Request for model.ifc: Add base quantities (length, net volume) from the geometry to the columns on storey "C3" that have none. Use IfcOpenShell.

First a look at what the model holds.

```python
import ifcopenshell
import ifcopenshell.util.element
import ifcopenshell.util.unit

model = ifcopenshell.open("model.ifc")
print(model.schema)
for unit_type in ("LENGTHUNIT", "AREAUNIT", "VOLUMEUNIT"):
    print(unit_type, ifcopenshell.util.unit.calculate_unit_scale(model, unit_type))
storey = next(s for s in model.by_type("IfcBuildingStorey") if s.Name == "C3")
columns = [e for e in ifcopenshell.util.element.get_decomposition(storey) if e.is_a("IfcColumn")]
for e in sorted(columns, key=lambda e: e.id()):
    print(e.id(), e.is_a(), e.Name, list(ifcopenshell.util.element.get_psets(e, qtos_only=True)), sep=" | ")
```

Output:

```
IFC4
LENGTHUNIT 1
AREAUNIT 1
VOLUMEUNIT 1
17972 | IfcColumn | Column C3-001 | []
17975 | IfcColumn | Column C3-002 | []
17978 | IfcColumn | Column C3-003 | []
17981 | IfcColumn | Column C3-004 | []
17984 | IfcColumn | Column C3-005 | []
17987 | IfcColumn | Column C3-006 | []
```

```python
import ifcopenshell
import ifcopenshell.api.pset
import ifcopenshell.geom
import ifcopenshell.util.element
import ifcopenshell.util.shape
import ifcopenshell.util.unit

model = ifcopenshell.open("model.ifc")
unit_scale = ifcopenshell.util.unit.calculate_unit_scale(model)
volume_scale = ifcopenshell.util.unit.calculate_unit_scale(model, "VOLUMEUNIT")
settings = ifcopenshell.geom.settings()

storey = next(s for s in model.by_type("IfcBuildingStorey") if s.Name == "C3")
columns = [e for e in ifcopenshell.util.element.get_decomposition(storey) if e.is_a("IfcColumn")]

for e in sorted(columns, key=lambda e: e.id()):
    if ifcopenshell.util.element.get_psets(e, qtos_only=True, should_inherit=False):
        continue
    # Geometry comes back in metres, in the element's own axes.
    shape = ifcopenshell.geom.create_shape(settings, e)
    values = {
        "Length": ifcopenshell.util.shape.get_z(shape.geometry) / unit_scale,
        "NetVolume": ifcopenshell.util.shape.get_volume(shape.geometry) / volume_scale,
    }
    qto = ifcopenshell.api.pset.add_qto(model, product=e, name="Qto_ColumnBaseQuantities")
    ifcopenshell.api.pset.edit_qto(model, qto=qto, properties=values)
    print(e.id(), {k: round(v, 3) for k, v in values.items()})

model.write("model_edited.ifc")
```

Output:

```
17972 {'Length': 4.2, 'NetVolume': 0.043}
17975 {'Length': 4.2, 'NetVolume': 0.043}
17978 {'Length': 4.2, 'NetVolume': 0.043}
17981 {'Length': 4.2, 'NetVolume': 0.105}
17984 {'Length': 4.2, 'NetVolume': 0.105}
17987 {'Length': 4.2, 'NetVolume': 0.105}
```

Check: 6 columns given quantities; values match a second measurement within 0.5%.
